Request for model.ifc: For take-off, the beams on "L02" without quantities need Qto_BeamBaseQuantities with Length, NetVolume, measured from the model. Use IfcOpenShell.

First a look at what the model holds.

```python
import ifcopenshell
import ifcopenshell.util.element
import ifcopenshell.util.unit

model = ifcopenshell.open("model.ifc")
print(model.schema)
for unit_type in ("LENGTHUNIT", "AREAUNIT", "VOLUMEUNIT"):
    print(unit_type, ifcopenshell.util.unit.calculate_unit_scale(model, unit_type))
storey = next(s for s in model.by_type("IfcBuildingStorey") if s.Name == "L02")
beams = [e for e in ifcopenshell.util.element.get_decomposition(storey) if e.is_a("IfcBeam")]
for e in sorted(beams, key=lambda e: e.id()):
    print(e.id(), e.is_a(), e.Name, list(ifcopenshell.util.element.get_psets(e, qtos_only=True)), sep=" | ")
```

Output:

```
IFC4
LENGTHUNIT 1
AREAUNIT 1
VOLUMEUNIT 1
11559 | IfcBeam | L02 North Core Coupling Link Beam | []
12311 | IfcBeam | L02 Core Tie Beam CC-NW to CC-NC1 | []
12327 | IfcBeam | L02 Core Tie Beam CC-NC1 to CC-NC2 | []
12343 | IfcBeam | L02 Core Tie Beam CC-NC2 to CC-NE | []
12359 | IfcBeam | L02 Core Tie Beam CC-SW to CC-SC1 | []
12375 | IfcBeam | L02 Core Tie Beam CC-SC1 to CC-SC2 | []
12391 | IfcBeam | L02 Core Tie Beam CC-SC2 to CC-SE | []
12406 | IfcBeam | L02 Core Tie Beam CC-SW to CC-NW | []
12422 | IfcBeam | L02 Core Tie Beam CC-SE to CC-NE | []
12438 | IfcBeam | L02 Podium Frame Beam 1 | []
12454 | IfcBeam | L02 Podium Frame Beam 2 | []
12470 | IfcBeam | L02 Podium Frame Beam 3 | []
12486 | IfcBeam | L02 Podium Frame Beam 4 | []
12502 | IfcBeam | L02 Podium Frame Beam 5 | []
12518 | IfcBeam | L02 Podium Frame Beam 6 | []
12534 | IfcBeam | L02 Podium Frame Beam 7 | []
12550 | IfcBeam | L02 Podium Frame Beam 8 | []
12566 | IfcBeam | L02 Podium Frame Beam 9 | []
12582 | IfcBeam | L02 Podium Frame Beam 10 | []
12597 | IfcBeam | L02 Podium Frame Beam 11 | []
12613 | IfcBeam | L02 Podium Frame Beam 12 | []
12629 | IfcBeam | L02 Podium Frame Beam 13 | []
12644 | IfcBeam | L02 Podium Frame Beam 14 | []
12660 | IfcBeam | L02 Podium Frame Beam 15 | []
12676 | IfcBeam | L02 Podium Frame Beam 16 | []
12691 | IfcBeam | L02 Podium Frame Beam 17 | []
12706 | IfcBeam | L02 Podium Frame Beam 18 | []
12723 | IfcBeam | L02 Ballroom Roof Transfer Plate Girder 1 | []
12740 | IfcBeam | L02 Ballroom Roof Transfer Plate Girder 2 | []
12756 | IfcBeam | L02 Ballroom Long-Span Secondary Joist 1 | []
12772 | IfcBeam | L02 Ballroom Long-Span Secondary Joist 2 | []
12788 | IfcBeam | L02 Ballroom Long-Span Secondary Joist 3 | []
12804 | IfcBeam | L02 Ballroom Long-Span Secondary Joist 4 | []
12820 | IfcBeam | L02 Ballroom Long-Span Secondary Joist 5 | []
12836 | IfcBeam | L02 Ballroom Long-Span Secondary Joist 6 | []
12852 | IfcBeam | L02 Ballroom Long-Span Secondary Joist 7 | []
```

```python
import ifcopenshell
import ifcopenshell.api.pset
import ifcopenshell.geom
import ifcopenshell.util.element
import ifcopenshell.util.shape
import ifcopenshell.util.unit

model = ifcopenshell.open("model.ifc")
unit_scale = ifcopenshell.util.unit.calculate_unit_scale(model)
volume_scale = ifcopenshell.util.unit.calculate_unit_scale(model, "VOLUMEUNIT")
settings = ifcopenshell.geom.settings()

storey = next(s for s in model.by_type("IfcBuildingStorey") if s.Name == "L02")
beams = [e for e in ifcopenshell.util.element.get_decomposition(storey) if e.is_a("IfcBeam")]

for e in sorted(beams, key=lambda e: e.id()):
    if ifcopenshell.util.element.get_psets(e, qtos_only=True, should_inherit=False):
        continue
    # Geometry comes back in metres, in the element's own axes.
    shape = ifcopenshell.geom.create_shape(settings, e)
    values = {
        "Length": ifcopenshell.util.shape.get_max_xyz(shape.geometry) / unit_scale,
        "NetVolume": ifcopenshell.util.shape.get_volume(shape.geometry) / volume_scale,
    }
    qto = ifcopenshell.api.pset.add_qto(model, product=e, name="Qto_BeamBaseQuantities")
    ifcopenshell.api.pset.edit_qto(model, qto=qto, properties=values)
    print(e.id(), {k: round(v, 3) for k, v in values.items()})

model.write("model_rev.ifc")
```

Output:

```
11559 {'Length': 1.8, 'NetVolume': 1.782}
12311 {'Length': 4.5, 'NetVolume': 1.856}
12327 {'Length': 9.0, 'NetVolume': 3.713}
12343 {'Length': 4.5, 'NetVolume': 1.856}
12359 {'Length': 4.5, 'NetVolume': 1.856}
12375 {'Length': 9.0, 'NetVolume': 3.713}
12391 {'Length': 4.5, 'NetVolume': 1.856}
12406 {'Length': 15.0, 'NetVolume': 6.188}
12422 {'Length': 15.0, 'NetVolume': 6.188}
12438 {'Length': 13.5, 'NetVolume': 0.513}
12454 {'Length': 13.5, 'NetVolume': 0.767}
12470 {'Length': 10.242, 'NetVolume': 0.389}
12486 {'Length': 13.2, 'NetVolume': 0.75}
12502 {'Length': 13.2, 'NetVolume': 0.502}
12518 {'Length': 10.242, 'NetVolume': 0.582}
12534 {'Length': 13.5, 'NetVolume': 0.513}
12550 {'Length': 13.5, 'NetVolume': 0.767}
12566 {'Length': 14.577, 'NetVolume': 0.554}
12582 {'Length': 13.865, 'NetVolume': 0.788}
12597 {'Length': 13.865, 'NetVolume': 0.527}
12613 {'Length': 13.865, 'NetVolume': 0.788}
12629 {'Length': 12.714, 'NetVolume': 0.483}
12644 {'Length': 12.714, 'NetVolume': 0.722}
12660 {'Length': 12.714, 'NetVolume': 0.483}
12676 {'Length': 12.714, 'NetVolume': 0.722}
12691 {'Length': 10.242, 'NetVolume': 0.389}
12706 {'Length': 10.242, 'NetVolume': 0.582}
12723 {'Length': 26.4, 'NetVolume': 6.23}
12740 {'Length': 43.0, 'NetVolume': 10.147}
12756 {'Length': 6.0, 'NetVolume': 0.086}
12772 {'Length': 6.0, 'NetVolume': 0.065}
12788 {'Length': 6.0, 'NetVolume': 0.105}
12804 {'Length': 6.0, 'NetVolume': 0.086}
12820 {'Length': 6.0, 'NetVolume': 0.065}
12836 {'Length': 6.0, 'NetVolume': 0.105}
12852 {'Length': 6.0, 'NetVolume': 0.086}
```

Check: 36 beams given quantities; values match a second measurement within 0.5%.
